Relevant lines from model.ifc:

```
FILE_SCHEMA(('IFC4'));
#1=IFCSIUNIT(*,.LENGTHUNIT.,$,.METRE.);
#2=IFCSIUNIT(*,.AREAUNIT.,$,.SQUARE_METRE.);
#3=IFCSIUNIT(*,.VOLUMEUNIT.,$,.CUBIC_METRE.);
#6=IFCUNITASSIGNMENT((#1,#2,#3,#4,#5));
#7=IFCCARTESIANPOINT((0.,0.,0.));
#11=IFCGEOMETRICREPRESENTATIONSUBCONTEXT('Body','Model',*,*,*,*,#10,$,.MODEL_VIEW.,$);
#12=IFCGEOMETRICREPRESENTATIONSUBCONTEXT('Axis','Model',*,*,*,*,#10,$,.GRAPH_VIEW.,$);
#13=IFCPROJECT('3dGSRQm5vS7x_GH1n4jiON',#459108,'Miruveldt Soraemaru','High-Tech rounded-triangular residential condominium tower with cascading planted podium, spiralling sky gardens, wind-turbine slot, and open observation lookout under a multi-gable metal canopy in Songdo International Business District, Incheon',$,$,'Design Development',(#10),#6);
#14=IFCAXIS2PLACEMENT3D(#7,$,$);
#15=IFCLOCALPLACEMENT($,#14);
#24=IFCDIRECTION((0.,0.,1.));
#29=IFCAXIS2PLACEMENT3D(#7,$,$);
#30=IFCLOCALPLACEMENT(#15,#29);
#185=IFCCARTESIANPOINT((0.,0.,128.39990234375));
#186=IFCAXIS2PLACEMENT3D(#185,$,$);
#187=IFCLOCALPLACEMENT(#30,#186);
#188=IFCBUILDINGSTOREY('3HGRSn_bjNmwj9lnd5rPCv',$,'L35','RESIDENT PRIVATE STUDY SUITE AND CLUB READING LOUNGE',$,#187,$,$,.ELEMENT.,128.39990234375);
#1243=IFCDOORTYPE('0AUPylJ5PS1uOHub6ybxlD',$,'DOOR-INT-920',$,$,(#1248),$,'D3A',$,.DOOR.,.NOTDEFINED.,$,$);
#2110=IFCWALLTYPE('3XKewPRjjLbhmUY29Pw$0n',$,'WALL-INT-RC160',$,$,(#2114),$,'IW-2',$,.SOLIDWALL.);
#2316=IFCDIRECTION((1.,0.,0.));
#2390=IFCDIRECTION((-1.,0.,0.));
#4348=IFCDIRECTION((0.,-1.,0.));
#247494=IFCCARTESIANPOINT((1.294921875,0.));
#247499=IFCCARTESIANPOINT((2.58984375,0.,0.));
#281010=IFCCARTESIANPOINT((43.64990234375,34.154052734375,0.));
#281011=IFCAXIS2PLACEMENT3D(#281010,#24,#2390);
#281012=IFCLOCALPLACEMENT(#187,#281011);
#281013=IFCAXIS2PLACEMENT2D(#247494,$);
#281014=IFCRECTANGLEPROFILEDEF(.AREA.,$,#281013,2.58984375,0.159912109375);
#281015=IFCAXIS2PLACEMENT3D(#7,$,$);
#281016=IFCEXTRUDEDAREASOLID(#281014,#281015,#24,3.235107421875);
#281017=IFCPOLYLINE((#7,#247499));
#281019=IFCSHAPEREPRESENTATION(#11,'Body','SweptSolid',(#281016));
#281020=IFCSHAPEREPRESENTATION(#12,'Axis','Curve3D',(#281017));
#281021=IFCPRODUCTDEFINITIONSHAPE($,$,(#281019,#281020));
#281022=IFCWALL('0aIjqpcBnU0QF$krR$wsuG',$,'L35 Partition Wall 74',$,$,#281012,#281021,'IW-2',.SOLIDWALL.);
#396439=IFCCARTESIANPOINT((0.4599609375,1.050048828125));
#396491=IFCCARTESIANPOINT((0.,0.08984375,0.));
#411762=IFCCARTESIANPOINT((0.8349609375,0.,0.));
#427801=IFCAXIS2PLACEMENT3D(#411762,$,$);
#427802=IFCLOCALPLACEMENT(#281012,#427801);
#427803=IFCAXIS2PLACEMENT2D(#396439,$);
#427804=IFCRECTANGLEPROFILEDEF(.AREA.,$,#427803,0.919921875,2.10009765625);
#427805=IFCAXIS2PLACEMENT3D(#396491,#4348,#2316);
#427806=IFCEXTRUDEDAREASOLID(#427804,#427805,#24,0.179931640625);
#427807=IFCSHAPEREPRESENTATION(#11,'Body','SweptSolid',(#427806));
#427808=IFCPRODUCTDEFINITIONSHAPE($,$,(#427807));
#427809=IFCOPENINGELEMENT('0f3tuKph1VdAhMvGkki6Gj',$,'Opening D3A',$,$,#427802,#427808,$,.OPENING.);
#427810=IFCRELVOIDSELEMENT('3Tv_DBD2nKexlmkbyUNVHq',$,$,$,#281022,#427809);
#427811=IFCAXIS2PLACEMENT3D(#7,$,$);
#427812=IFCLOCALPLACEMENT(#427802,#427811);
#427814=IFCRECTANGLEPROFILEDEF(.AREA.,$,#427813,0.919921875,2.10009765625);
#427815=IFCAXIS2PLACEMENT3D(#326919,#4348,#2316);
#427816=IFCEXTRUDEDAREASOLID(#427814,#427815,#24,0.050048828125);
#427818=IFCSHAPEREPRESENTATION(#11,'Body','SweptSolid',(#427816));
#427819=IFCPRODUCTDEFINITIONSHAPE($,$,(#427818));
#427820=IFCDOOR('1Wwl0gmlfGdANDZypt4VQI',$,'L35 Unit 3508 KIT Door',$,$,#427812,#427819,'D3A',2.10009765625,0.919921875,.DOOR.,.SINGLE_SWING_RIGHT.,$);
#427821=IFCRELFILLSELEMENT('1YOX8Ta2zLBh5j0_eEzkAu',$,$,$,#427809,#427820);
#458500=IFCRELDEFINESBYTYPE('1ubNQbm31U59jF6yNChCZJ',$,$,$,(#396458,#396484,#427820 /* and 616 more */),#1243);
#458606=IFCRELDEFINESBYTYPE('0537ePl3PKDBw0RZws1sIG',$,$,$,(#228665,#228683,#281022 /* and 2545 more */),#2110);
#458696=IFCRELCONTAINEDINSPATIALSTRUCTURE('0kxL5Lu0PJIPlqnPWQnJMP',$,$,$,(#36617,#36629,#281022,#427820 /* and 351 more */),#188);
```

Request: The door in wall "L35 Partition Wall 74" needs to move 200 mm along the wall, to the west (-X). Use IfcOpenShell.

```python
import ifcopenshell
import ifcopenshell.api.geometry
import ifcopenshell.util.placement
import ifcopenshell.util.unit

model = ifcopenshell.open("model.ifc")
unit_scale = ifcopenshell.util.unit.calculate_unit_scale(model)

door = model.by_guid("1Wwl0gmlfGdANDZypt4VQI")
opening = door.FillsVoids[0].RelatingOpeningElement
wall = opening.VoidsElements[0].RelatingBuildingElement

wall_matrix = ifcopenshell.util.placement.get_local_placement(wall.ObjectPlacement)
shift = wall_matrix[:3, 0] * 0.2 / unit_scale
before = ifcopenshell.util.placement.get_local_placement(door.ObjectPlacement)[:3, 3].copy()

# The door is placed relative to its opening, so it follows when the opening moves.
matrix = ifcopenshell.util.placement.get_local_placement(opening.ObjectPlacement)
matrix[:3, 3] += shift
ifcopenshell.api.geometry.edit_object_placement(
    model, product=opening, matrix=matrix, is_si=False, should_transform_children=True
)

after = ifcopenshell.util.placement.get_local_placement(door.ObjectPlacement)[:3, 3]
print("door moved by", (after - before).round(3) + 0.0)

model.write("model-out.ifc")
```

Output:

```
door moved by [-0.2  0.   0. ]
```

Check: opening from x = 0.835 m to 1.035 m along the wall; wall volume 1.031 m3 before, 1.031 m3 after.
